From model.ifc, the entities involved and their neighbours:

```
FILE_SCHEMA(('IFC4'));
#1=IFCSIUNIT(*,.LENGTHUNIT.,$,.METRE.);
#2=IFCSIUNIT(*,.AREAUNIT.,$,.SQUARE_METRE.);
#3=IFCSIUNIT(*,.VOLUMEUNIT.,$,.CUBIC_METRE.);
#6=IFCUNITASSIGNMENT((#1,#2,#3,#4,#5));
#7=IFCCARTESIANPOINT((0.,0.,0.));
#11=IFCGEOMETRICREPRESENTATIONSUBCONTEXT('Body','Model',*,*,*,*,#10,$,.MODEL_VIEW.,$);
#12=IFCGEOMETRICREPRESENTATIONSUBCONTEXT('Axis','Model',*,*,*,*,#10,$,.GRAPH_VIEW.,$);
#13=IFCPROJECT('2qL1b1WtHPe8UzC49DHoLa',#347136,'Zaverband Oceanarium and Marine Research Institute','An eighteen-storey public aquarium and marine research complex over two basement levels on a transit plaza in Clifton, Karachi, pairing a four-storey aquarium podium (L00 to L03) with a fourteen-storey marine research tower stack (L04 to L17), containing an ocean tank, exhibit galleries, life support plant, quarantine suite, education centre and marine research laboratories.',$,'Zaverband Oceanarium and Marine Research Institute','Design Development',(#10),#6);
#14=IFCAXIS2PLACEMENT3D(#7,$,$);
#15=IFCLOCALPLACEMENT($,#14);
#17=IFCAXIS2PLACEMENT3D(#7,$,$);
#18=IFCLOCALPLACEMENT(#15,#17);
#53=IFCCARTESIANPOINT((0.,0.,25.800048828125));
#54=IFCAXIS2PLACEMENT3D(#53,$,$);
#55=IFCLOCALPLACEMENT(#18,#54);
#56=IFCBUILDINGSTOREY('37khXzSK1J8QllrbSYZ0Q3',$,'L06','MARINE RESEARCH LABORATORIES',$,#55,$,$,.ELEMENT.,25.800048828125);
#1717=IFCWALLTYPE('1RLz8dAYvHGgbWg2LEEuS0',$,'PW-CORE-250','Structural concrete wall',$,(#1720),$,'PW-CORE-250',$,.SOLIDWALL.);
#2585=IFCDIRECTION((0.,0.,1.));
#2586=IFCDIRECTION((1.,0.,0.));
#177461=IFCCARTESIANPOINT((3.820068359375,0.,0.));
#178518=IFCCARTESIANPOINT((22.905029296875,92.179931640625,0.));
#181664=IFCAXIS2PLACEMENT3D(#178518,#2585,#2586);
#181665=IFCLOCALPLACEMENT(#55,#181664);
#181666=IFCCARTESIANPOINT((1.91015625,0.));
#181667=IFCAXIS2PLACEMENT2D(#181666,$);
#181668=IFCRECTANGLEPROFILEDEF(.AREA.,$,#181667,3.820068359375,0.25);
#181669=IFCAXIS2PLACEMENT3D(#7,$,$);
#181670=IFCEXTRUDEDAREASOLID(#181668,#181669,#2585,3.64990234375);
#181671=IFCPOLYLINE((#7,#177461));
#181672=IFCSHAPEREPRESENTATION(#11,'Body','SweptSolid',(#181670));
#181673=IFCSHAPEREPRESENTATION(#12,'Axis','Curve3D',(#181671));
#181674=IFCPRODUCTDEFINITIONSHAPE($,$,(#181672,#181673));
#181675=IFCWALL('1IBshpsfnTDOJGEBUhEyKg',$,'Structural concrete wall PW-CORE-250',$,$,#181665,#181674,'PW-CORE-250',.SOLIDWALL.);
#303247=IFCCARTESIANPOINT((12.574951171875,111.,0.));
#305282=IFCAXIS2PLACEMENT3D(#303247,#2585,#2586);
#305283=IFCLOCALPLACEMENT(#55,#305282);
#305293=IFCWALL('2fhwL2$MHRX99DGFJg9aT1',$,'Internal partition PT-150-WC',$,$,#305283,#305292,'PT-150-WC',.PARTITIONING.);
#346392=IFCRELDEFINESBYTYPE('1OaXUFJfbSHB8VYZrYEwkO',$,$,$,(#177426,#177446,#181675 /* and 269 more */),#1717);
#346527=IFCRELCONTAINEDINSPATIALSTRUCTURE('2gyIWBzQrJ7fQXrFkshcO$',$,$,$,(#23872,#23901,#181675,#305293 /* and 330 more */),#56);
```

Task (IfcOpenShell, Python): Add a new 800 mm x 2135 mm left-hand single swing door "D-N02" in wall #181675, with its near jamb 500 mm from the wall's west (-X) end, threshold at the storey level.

```python
import numpy as np
import ifcopenshell
import ifcopenshell.api.feature
import ifcopenshell.api.geometry
import ifcopenshell.api.root
import ifcopenshell.api.spatial
import ifcopenshell.geom
import ifcopenshell.util.element
import ifcopenshell.util.placement
import ifcopenshell.util.representation
import ifcopenshell.util.shape
import ifcopenshell.util.unit

model = ifcopenshell.open("model.ifc")
unit_scale = ifcopenshell.util.unit.calculate_unit_scale(model)
settings = ifcopenshell.geom.settings()


def volume(element):
    """Net volume in cubic metres, openings subtracted."""
    shape = ifcopenshell.geom.create_shape(settings, element)
    return ifcopenshell.util.shape.get_volume(shape.geometry)


wall = model.by_guid("1IBshpsfnTDOJGEBUhEyKg")
storey = ifcopenshell.util.element.get_container(wall, ifc_class="IfcBuildingStorey")
context = ifcopenshell.util.representation.get_context(model, "Model", "Body", "MODEL_VIEW")
before = volume(wall)

width, height, from_end, sill = 0.8, 2.135, 0.5, 0.0  # metres

# The wall runs along its own X axis, and the end named is its -X end.
wall_shape = ifcopenshell.geom.create_shape(settings, wall)
x, y, z = ifcopenshell.util.shape.get_vertices(wall_shape.geometry).T
start = x.min() + from_end
face, thickness = float(y.min()), float(y.max() - y.min())
wall_matrix = ifcopenshell.util.placement.get_local_placement(wall.ObjectPlacement)
level = ifcopenshell.util.placement.get_local_placement(storey.ObjectPlacement)[2, 3]


def in_wall(x, y):
    """Placement at x, y metres in the wall's axes, at sill height."""
    matrix = wall_matrix.copy()
    matrix[:, 3] = wall_matrix @ np.array([x / unit_scale, y / unit_scale, 0.0, 1.0])
    matrix[2, 3] = level + sill / unit_scale
    return matrix


# Opening: a box that overshoots both wall faces by 50 mm.
opening = ifcopenshell.api.root.create_entity(model, ifc_class="IfcOpeningElement", predefined_type="OPENING")
box = ifcopenshell.api.geometry.add_wall_representation(
    model, context=context, length=width, height=height, thickness=thickness + 0.1
)
ifcopenshell.api.geometry.assign_representation(model, product=opening, representation=box)
ifcopenshell.api.geometry.edit_object_placement(model, product=opening, matrix=in_wall(start, face - 0.05), is_si=False)
ifcopenshell.api.feature.add_feature(model, feature=opening, element=wall)

door = ifcopenshell.api.root.create_entity(model, ifc_class="IfcDoor", name="D-N02", predefined_type="DOOR")
door.OverallWidth, door.OverallHeight = width / unit_scale, height / unit_scale
door.OperationType = "SINGLE_SWING_LEFT"
body = ifcopenshell.api.geometry.add_door_representation(
    model,
    context=context,
    overall_width=door.OverallWidth,
    overall_height=door.OverallHeight,
    operation_type="SINGLE_SWING_LEFT",
    lining_properties={"LiningDepth": thickness / unit_scale, "ThresholdDepth": thickness / unit_scale},
)
ifcopenshell.api.geometry.assign_representation(model, product=door, representation=body)
ifcopenshell.api.spatial.assign_container(model, products=[door], relating_structure=storey)
ifcopenshell.api.feature.add_filling(model, opening=opening, element=door)

# The lining spans the wall, so the door starts at the wall face.
ifcopenshell.api.geometry.edit_object_placement(model, product=door, matrix=in_wall(start, face), is_si=False)

after = volume(wall)

print(f"wall volume {before:.3f} -> {after:.3f} m3")

model.write("model_v2.ifc")
```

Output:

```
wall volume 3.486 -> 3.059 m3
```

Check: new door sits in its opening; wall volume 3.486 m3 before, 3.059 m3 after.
